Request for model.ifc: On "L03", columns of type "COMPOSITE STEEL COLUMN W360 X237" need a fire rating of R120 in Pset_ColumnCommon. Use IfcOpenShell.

First a look at what the model holds.

```python
import ifcopenshell
import ifcopenshell.util.element

model = ifcopenshell.open("model.ifc")
print(model.schema)
storey = next(s for s in model.by_type("IfcBuildingStorey") if s.Name == "L03")
columns = [e for e in ifcopenshell.util.element.get_decomposition(storey) if e.is_a("IfcColumn")]
seen = {}
for e in columns:
    element_type = ifcopenshell.util.element.get_type(e)
    key = (element_type.Name if element_type != e and element_type else None, ifcopenshell.util.element.get_pset(e, "Pset_ColumnCommon", "FireRating"))
    seen[key] = seen.get(key, 0) + 1
for (name, value), count in sorted(seen.items(), key=str):
    print(count, "x", name, "|", value)
```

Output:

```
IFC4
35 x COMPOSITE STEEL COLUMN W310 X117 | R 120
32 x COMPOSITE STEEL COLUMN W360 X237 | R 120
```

```python
import ifcopenshell
import ifcopenshell.api.pset
import ifcopenshell.util.element

model = ifcopenshell.open("model.ifc")

storey = next(s for s in model.by_type("IfcBuildingStorey") if s.Name == "L03")
columns = [e for e in ifcopenshell.util.element.get_decomposition(storey) if e.is_a("IfcColumn")]

count = 0
for e in columns:
    element_type = ifcopenshell.util.element.get_type(e)
    if element_type in (None, e) or element_type.Name != "COMPOSITE STEEL COLUMN W360 X237":
        continue
    # add_pset returns the element's existing set when there is one.
    pset = ifcopenshell.api.pset.add_pset(model, product=e, name="Pset_ColumnCommon")
    ifcopenshell.api.pset.edit_pset(model, pset=pset, properties={"FireRating": "R120"})
    count += 1

print(count, "columns updated")

model.write("model-out.ifc")
```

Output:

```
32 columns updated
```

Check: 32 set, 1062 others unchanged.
